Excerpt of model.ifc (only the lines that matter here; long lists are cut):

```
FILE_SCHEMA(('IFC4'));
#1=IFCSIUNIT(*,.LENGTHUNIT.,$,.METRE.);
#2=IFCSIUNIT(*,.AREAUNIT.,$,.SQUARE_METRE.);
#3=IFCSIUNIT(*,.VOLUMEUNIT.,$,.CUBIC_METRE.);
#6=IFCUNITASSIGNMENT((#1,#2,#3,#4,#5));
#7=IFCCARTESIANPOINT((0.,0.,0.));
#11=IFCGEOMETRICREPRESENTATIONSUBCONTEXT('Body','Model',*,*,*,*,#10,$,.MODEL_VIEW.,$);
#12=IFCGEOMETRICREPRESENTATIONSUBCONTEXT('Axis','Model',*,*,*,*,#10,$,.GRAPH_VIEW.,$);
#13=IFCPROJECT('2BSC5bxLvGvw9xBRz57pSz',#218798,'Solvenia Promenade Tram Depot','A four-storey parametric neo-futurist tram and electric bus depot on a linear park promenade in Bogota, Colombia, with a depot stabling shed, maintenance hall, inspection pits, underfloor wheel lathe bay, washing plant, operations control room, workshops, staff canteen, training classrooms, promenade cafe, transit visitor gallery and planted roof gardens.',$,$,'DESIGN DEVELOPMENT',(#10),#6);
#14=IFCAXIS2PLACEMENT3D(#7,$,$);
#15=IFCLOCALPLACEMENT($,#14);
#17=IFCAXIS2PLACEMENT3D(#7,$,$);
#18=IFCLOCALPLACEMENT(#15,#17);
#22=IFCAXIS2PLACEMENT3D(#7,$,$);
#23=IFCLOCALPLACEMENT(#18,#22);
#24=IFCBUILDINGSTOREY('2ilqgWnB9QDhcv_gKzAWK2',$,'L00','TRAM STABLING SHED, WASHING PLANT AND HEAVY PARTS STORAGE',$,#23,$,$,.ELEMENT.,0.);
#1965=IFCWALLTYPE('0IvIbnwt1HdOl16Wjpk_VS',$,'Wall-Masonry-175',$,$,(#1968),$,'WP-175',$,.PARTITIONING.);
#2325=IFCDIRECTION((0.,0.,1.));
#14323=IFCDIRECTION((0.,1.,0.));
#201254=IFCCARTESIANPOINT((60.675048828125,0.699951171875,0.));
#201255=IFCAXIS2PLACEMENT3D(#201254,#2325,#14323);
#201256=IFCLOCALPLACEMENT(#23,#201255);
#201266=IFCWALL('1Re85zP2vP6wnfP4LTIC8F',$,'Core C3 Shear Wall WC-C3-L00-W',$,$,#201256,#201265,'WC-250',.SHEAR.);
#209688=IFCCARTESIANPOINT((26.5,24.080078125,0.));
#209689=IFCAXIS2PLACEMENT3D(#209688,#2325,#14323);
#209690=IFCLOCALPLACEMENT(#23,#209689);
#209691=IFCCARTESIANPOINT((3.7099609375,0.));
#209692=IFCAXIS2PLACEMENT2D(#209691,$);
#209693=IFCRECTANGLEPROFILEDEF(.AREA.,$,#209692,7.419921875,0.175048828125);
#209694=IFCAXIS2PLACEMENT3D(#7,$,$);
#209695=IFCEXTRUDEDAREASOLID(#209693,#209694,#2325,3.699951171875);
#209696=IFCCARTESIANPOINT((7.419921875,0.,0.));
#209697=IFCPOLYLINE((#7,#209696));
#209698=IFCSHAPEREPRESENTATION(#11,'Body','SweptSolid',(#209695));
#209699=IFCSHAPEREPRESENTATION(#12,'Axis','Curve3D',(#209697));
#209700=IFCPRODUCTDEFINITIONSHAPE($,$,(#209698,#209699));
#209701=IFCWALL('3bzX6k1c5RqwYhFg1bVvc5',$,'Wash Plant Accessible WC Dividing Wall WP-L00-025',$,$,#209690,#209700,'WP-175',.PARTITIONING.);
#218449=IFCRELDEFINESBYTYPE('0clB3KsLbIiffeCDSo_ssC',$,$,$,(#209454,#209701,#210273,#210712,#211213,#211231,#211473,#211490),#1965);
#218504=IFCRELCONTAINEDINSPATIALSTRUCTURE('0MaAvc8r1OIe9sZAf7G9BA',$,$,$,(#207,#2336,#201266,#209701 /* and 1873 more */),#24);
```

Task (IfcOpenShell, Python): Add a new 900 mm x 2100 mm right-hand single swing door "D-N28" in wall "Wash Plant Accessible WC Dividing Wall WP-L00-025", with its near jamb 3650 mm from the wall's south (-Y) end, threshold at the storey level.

```python
import numpy as np
import ifcopenshell
import ifcopenshell.api.feature
import ifcopenshell.api.geometry
import ifcopenshell.api.root
import ifcopenshell.api.spatial
import ifcopenshell.geom
import ifcopenshell.util.element
import ifcopenshell.util.placement
import ifcopenshell.util.representation
import ifcopenshell.util.shape
import ifcopenshell.util.unit

model = ifcopenshell.open("model.ifc")
unit_scale = ifcopenshell.util.unit.calculate_unit_scale(model)
settings = ifcopenshell.geom.settings()


def volume(element):
    """Net volume in cubic metres, openings subtracted."""
    shape = ifcopenshell.geom.create_shape(settings, element)
    return ifcopenshell.util.shape.get_volume(shape.geometry)


wall = model.by_guid("3bzX6k1c5RqwYhFg1bVvc5")
storey = ifcopenshell.util.element.get_container(wall, ifc_class="IfcBuildingStorey")
context = ifcopenshell.util.representation.get_context(model, "Model", "Body", "MODEL_VIEW")
before = volume(wall)

width, height, from_end, sill = 0.9, 2.1, 3.65, 0.0  # metres

# The wall runs along its own X axis, and the end named is its -X end.
wall_shape = ifcopenshell.geom.create_shape(settings, wall)
x, y, z = ifcopenshell.util.shape.get_vertices(wall_shape.geometry).T
start = x.min() + from_end
face, thickness = float(y.min()), float(y.max() - y.min())
wall_matrix = ifcopenshell.util.placement.get_local_placement(wall.ObjectPlacement)
level = ifcopenshell.util.placement.get_local_placement(storey.ObjectPlacement)[2, 3]


def in_wall(x, y):
    """Placement at x, y metres in the wall's axes, at sill height."""
    matrix = wall_matrix.copy()
    matrix[:, 3] = wall_matrix @ np.array([x / unit_scale, y / unit_scale, 0.0, 1.0])
    matrix[2, 3] = level + sill / unit_scale
    return matrix


# Opening: a box that overshoots both wall faces by 50 mm.
opening = ifcopenshell.api.root.create_entity(model, ifc_class="IfcOpeningElement", predefined_type="OPENING")
box = ifcopenshell.api.geometry.add_wall_representation(
    model, context=context, length=width, height=height, thickness=thickness + 0.1
)
ifcopenshell.api.geometry.assign_representation(model, product=opening, representation=box)
ifcopenshell.api.geometry.edit_object_placement(model, product=opening, matrix=in_wall(start, face - 0.05), is_si=False)
ifcopenshell.api.feature.add_feature(model, feature=opening, element=wall)

door = ifcopenshell.api.root.create_entity(model, ifc_class="IfcDoor", name="D-N28", predefined_type="DOOR")
door.OverallWidth, door.OverallHeight = width / unit_scale, height / unit_scale
door.OperationType = "SINGLE_SWING_RIGHT"
body = ifcopenshell.api.geometry.add_door_representation(
    model,
    context=context,
    overall_width=door.OverallWidth,
    overall_height=door.OverallHeight,
    operation_type="SINGLE_SWING_RIGHT",
    lining_properties={"LiningDepth": thickness / unit_scale, "ThresholdDepth": thickness / unit_scale},
)
ifcopenshell.api.geometry.assign_representation(model, product=door, representation=body)
ifcopenshell.api.spatial.assign_container(model, products=[door], relating_structure=storey)
ifcopenshell.api.feature.add_filling(model, opening=opening, element=door)

# The lining spans the wall, so the door starts at the wall face.
ifcopenshell.api.geometry.edit_object_placement(model, product=door, matrix=in_wall(start, face), is_si=False)

after = volume(wall)

print(f"wall volume {before:.3f} -> {after:.3f} m3")

model.write("model_rev.ifc")
```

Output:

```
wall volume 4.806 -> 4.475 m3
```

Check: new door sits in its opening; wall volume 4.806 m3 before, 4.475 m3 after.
